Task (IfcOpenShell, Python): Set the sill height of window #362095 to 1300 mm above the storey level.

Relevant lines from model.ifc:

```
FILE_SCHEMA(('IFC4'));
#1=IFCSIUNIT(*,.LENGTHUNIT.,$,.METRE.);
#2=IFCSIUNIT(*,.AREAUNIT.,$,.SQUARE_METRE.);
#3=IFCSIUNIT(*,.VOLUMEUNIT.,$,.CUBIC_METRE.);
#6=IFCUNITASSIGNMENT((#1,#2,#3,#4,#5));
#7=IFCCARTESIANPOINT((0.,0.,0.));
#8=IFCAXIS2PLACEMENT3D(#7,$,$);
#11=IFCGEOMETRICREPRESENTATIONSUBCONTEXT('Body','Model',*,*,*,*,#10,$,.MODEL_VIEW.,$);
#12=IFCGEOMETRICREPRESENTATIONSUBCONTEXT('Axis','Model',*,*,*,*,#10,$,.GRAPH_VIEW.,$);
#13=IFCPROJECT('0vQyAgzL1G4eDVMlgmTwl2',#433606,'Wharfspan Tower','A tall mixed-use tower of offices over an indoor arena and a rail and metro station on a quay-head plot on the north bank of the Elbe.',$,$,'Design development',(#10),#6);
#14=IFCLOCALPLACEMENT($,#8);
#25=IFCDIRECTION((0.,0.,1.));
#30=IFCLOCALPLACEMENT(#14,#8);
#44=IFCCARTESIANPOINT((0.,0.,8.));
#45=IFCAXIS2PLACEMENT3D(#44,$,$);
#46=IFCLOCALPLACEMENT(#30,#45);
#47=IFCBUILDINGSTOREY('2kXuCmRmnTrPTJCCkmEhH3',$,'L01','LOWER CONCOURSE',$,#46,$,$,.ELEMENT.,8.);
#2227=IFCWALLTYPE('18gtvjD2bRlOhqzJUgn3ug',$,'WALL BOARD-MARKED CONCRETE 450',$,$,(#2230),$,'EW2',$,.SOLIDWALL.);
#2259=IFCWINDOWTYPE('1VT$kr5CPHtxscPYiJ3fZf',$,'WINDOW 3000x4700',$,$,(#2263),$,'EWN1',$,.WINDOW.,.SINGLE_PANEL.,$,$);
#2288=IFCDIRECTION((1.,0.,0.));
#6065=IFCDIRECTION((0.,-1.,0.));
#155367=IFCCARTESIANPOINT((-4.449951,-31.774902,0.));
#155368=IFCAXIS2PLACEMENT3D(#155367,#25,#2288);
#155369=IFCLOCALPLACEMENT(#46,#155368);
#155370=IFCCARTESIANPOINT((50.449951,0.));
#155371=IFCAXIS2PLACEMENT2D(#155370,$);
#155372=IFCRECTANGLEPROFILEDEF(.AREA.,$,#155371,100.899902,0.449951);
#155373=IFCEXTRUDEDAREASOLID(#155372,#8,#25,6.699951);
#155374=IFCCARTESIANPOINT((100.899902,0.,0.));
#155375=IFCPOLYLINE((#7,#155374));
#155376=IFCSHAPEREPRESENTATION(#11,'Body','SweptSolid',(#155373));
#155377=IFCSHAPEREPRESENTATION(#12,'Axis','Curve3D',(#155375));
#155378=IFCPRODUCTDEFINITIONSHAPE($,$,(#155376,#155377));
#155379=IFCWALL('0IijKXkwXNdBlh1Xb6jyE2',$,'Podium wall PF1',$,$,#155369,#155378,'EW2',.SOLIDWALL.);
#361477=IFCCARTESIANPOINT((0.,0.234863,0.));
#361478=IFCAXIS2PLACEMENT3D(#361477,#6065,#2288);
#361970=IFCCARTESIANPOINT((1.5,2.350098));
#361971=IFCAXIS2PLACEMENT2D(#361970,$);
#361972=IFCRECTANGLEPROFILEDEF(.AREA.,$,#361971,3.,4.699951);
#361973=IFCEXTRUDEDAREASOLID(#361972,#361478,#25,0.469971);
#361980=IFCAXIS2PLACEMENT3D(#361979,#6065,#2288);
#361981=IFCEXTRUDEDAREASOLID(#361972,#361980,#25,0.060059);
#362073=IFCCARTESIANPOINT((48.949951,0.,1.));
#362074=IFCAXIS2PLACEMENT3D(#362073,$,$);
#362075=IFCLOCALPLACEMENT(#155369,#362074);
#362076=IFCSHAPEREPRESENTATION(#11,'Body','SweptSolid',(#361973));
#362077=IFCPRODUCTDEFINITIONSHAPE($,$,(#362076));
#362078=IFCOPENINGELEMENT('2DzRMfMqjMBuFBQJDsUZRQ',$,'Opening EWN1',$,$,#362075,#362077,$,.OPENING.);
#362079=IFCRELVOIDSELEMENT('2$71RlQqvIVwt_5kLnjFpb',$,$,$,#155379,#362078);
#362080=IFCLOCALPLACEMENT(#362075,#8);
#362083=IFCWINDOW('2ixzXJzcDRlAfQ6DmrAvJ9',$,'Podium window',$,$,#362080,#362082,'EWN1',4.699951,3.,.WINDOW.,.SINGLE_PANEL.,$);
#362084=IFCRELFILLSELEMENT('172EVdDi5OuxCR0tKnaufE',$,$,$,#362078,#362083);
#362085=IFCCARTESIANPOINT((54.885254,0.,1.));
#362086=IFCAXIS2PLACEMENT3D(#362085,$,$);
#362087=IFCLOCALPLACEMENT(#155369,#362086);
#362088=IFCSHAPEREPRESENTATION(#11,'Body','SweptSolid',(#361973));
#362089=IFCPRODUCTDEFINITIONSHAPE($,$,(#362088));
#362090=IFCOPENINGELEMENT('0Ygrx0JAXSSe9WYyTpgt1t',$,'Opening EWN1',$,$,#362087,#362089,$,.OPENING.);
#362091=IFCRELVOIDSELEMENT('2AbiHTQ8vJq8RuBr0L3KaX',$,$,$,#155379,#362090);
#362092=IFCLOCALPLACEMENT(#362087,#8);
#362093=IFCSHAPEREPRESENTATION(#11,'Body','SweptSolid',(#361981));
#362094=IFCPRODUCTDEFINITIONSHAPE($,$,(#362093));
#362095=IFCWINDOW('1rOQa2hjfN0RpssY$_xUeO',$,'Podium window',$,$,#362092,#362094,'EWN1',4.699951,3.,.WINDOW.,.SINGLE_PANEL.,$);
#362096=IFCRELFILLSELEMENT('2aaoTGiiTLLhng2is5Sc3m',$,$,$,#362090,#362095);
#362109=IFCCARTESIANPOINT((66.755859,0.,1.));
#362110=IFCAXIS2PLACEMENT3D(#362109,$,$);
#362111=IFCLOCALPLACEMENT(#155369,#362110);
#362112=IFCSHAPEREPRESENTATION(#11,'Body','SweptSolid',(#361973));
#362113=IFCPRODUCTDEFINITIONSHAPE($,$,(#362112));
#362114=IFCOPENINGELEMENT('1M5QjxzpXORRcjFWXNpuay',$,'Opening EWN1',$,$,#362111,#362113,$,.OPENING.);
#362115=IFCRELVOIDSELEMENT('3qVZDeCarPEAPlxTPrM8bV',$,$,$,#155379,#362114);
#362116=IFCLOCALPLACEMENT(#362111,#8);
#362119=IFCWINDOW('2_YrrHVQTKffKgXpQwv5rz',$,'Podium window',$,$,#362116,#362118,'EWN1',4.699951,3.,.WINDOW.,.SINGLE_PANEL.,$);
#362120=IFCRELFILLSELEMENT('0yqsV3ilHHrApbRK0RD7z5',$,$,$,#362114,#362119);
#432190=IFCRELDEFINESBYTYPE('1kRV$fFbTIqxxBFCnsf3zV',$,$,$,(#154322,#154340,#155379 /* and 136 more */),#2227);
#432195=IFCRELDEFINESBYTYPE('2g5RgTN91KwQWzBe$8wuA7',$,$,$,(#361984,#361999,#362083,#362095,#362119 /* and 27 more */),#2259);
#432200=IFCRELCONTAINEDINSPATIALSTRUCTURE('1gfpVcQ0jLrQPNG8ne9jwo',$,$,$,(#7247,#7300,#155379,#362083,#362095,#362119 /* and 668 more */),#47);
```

```python
import numpy as np
import ifcopenshell
import ifcopenshell.api.geometry
import ifcopenshell.geom
import ifcopenshell.util.element
import ifcopenshell.util.placement
import ifcopenshell.util.shape
import ifcopenshell.util.unit

model = ifcopenshell.open("model.ifc")
unit_scale = ifcopenshell.util.unit.calculate_unit_scale(model)

window = model.by_id(362095)
opening = window.FillsVoids[0].RelatingOpeningElement
storey = ifcopenshell.util.element.get_container(window, ifc_class="IfcBuildingStorey")
level = ifcopenshell.util.placement.get_local_placement(storey.ObjectPlacement)[2, 3]

# The opening's origin need not be at the sill, so measure its lowest point.
shape = ifcopenshell.geom.create_shape(ifcopenshell.geom.settings(), opening)
bottom = ifcopenshell.util.shape.get_shape_bottom_elevation(shape, shape.geometry) / unit_scale
dz = level + 1.3 / unit_scale - bottom

shift = np.array([0.0, 0.0, dz])
# The window is placed relative to its opening, so it follows when the opening moves.
matrix = ifcopenshell.util.placement.get_local_placement(opening.ObjectPlacement)
matrix[:3, 3] += shift
ifcopenshell.api.geometry.edit_object_placement(
    model, product=opening, matrix=matrix, is_si=False, should_transform_children=True
)

print(f"moved by {dz * unit_scale:+.3f} m")

model.write("model_updated.ifc")
```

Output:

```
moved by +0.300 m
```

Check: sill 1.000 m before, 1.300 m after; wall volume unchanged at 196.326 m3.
